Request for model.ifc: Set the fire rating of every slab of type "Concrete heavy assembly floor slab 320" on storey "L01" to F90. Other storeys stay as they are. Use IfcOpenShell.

First a look at what the model holds.

```python
import ifcopenshell
import ifcopenshell.util.element

model = ifcopenshell.open("model.ifc")
print(model.schema)
storey = next(s for s in model.by_type("IfcBuildingStorey") if s.Name == "L01")
slabs = [e for e in ifcopenshell.util.element.get_decomposition(storey) if e.is_a("IfcSlab")]
seen = {}
for e in slabs:
    element_type = ifcopenshell.util.element.get_type(e)
    key = (element_type.Name if element_type != e and element_type else None, ifcopenshell.util.element.get_pset(e, "Pset_SlabCommon", "FireRating"))
    seen[key] = seen.get(key, 0) + 1
for (name, value), count in sorted(seen.items(), key=str):
    print(count, "x", name, "|", value)
```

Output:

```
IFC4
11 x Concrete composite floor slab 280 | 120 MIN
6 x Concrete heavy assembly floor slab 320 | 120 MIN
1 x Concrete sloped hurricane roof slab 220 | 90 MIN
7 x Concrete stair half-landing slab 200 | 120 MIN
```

```python
import ifcopenshell
import ifcopenshell.api.pset
import ifcopenshell.util.element

model = ifcopenshell.open("model.ifc")

storey = next(s for s in model.by_type("IfcBuildingStorey") if s.Name == "L01")
slabs = [e for e in ifcopenshell.util.element.get_decomposition(storey) if e.is_a("IfcSlab")]

count = 0
for e in slabs:
    element_type = ifcopenshell.util.element.get_type(e)
    if element_type in (None, e) or element_type.Name != "Concrete heavy assembly floor slab 320":
        continue
    # add_pset returns the element's existing set when there is one.
    pset = ifcopenshell.api.pset.add_pset(model, product=e, name="Pset_SlabCommon")
    ifcopenshell.api.pset.edit_pset(model, pset=pset, properties={"FireRating": "F90"})
    count += 1

print(count, "slabs updated")

model.write("model_edited.ifc")
```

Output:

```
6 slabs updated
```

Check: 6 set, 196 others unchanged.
